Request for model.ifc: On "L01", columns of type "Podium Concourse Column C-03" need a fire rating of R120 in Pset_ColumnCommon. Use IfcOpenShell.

First a look at what the model holds.

```python
import ifcopenshell
import ifcopenshell.util.element

model = ifcopenshell.open("model.ifc")
print(model.schema)
storey = next(s for s in model.by_type("IfcBuildingStorey") if s.Name == "L01")
columns = [e for e in ifcopenshell.util.element.get_decomposition(storey) if e.is_a("IfcColumn")]
seen = {}
for e in columns:
    element_type = ifcopenshell.util.element.get_type(e)
    key = (element_type.Name if element_type != e and element_type else None, ifcopenshell.util.element.get_pset(e, "Pset_ColumnCommon", "FireRating"))
    seen[key] = seen.get(key, 0) + 1
for (name, value), count in sorted(seen.items(), key=str):
    print(count, "x", name, "|", value)
```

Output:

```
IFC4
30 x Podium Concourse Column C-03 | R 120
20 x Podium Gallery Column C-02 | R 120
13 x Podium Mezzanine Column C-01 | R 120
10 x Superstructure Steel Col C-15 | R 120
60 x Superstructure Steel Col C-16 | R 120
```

```python
import ifcopenshell
import ifcopenshell.api.pset
import ifcopenshell.util.element

model = ifcopenshell.open("model.ifc")

storey = next(s for s in model.by_type("IfcBuildingStorey") if s.Name == "L01")
columns = [e for e in ifcopenshell.util.element.get_decomposition(storey) if e.is_a("IfcColumn")]

count = 0
for e in columns:
    element_type = ifcopenshell.util.element.get_type(e)
    if element_type in (None, e) or element_type.Name != "Podium Concourse Column C-03":
        continue
    # add_pset returns the element's existing set when there is one.
    pset = ifcopenshell.api.pset.add_pset(model, product=e, name="Pset_ColumnCommon")
    ifcopenshell.api.pset.edit_pset(model, pset=pset, properties={"FireRating": "R120"})
    count += 1

print(count, "columns updated")

model.write("model_rev.ifc")
```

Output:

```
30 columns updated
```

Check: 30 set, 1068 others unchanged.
